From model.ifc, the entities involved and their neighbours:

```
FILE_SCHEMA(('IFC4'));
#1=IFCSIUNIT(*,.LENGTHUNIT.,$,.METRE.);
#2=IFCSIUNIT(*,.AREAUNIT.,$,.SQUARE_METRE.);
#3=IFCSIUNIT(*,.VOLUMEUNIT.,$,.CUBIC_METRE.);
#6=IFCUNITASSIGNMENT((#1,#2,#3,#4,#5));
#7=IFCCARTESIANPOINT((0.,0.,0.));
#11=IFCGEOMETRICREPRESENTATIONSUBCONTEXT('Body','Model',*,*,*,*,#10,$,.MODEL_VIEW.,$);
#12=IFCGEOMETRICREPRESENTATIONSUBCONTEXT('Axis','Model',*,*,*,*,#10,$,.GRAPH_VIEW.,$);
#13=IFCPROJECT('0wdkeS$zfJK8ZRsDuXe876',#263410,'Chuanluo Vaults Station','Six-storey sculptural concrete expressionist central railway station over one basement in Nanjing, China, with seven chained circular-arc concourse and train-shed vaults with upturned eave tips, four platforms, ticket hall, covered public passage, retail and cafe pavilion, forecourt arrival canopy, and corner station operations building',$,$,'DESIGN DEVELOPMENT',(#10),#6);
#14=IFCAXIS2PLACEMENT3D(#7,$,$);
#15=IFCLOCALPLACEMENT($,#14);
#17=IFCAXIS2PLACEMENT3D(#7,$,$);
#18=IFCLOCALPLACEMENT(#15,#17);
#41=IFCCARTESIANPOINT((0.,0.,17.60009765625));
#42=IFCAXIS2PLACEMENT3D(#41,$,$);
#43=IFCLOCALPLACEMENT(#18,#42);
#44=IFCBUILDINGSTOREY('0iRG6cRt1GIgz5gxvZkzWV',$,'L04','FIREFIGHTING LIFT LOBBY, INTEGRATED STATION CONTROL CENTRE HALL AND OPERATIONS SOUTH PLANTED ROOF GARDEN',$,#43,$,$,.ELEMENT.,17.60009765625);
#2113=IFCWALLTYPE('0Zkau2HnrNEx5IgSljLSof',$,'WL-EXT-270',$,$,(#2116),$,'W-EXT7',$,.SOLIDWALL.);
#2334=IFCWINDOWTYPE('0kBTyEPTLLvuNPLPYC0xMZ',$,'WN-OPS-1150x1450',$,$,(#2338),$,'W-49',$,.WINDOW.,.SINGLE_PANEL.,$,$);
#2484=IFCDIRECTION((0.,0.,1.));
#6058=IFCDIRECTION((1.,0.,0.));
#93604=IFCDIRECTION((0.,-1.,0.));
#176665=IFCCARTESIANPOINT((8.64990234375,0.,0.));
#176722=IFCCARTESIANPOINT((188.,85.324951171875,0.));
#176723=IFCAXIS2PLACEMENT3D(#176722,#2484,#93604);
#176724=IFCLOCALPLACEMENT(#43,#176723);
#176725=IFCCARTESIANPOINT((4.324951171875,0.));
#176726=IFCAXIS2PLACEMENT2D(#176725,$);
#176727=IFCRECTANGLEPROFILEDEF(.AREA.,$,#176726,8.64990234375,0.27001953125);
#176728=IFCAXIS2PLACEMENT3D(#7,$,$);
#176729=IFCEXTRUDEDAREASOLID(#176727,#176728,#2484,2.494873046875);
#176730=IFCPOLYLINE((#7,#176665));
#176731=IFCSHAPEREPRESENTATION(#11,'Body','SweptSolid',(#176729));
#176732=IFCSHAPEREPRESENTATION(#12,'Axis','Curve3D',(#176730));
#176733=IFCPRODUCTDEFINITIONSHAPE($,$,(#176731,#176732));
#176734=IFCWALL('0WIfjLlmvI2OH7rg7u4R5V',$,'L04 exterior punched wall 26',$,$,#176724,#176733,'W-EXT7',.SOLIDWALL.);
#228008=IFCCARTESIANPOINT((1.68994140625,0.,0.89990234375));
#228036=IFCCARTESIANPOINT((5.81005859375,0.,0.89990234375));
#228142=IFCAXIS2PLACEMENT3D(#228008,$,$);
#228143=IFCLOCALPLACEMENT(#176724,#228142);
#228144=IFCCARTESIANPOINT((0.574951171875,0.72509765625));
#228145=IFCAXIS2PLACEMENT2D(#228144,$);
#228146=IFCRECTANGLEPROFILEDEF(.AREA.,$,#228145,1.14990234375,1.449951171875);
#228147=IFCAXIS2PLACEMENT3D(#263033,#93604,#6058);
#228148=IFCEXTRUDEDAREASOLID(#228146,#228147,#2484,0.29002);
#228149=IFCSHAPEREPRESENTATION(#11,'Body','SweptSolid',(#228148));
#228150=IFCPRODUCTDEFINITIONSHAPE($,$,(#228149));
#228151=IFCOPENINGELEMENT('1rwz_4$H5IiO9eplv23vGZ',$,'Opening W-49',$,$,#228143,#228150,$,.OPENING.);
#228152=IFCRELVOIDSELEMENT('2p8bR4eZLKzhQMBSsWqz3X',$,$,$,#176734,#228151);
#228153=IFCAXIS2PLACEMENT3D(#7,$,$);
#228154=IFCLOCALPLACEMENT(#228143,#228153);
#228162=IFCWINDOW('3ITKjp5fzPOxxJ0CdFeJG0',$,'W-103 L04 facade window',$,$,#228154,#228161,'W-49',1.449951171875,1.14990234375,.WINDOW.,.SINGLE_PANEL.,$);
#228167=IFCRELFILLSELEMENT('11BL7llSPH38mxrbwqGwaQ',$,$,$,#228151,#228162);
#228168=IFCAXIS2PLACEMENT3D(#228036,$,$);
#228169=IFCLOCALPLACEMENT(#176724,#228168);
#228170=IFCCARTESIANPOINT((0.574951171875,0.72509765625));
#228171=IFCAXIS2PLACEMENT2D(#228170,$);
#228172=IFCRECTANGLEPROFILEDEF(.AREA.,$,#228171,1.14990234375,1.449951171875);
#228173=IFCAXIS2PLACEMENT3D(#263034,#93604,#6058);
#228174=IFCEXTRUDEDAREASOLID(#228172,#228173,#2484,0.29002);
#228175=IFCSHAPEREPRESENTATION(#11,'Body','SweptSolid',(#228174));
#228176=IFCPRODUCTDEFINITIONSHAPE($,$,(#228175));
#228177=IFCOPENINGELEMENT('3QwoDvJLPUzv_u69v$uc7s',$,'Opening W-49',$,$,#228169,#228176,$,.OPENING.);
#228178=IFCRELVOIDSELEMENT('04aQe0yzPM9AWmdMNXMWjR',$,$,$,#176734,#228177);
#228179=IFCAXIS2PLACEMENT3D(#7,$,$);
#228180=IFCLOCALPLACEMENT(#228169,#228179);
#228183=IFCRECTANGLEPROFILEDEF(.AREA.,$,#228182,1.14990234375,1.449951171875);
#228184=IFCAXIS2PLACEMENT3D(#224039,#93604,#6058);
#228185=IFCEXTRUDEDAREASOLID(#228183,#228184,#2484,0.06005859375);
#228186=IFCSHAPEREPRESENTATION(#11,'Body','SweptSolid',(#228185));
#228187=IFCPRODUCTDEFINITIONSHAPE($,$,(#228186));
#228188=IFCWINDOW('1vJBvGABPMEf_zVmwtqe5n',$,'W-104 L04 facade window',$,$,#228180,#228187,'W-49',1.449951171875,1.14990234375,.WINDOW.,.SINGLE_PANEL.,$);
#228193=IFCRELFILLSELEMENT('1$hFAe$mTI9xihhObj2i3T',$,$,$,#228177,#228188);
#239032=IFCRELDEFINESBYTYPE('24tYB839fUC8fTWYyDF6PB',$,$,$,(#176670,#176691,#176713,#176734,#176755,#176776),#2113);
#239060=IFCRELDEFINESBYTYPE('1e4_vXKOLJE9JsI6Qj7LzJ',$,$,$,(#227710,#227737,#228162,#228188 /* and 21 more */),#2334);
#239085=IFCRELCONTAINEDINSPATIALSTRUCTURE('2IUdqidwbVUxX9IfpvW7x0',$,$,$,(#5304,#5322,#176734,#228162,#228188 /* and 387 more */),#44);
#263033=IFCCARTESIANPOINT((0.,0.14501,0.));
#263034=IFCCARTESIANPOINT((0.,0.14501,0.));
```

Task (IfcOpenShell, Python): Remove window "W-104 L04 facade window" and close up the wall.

```python
import ifcopenshell
import ifcopenshell.api.feature
import ifcopenshell.api.root
import ifcopenshell.geom
import ifcopenshell.util.shape

model = ifcopenshell.open("model.ifc")
settings = ifcopenshell.geom.settings()


def volume(element):
    """Net volume in cubic metres, openings subtracted."""
    shape = ifcopenshell.geom.create_shape(settings, element)
    return ifcopenshell.util.shape.get_volume(shape.geometry)


window = model.by_id(228188)
opening = window.FillsVoids[0].RelatingOpeningElement
wall = opening.VoidsElements[0].RelatingBuildingElement
before = volume(wall)

ifcopenshell.api.root.remove_product(model, product=window)
ifcopenshell.api.feature.remove_feature(model, feature=opening)

after = volume(wall)

print(f"wall volume {before:.3f} -> {after:.3f} m3")

model.write("model_v2.ifc")
```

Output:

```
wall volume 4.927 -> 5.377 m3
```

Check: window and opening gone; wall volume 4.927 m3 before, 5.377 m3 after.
